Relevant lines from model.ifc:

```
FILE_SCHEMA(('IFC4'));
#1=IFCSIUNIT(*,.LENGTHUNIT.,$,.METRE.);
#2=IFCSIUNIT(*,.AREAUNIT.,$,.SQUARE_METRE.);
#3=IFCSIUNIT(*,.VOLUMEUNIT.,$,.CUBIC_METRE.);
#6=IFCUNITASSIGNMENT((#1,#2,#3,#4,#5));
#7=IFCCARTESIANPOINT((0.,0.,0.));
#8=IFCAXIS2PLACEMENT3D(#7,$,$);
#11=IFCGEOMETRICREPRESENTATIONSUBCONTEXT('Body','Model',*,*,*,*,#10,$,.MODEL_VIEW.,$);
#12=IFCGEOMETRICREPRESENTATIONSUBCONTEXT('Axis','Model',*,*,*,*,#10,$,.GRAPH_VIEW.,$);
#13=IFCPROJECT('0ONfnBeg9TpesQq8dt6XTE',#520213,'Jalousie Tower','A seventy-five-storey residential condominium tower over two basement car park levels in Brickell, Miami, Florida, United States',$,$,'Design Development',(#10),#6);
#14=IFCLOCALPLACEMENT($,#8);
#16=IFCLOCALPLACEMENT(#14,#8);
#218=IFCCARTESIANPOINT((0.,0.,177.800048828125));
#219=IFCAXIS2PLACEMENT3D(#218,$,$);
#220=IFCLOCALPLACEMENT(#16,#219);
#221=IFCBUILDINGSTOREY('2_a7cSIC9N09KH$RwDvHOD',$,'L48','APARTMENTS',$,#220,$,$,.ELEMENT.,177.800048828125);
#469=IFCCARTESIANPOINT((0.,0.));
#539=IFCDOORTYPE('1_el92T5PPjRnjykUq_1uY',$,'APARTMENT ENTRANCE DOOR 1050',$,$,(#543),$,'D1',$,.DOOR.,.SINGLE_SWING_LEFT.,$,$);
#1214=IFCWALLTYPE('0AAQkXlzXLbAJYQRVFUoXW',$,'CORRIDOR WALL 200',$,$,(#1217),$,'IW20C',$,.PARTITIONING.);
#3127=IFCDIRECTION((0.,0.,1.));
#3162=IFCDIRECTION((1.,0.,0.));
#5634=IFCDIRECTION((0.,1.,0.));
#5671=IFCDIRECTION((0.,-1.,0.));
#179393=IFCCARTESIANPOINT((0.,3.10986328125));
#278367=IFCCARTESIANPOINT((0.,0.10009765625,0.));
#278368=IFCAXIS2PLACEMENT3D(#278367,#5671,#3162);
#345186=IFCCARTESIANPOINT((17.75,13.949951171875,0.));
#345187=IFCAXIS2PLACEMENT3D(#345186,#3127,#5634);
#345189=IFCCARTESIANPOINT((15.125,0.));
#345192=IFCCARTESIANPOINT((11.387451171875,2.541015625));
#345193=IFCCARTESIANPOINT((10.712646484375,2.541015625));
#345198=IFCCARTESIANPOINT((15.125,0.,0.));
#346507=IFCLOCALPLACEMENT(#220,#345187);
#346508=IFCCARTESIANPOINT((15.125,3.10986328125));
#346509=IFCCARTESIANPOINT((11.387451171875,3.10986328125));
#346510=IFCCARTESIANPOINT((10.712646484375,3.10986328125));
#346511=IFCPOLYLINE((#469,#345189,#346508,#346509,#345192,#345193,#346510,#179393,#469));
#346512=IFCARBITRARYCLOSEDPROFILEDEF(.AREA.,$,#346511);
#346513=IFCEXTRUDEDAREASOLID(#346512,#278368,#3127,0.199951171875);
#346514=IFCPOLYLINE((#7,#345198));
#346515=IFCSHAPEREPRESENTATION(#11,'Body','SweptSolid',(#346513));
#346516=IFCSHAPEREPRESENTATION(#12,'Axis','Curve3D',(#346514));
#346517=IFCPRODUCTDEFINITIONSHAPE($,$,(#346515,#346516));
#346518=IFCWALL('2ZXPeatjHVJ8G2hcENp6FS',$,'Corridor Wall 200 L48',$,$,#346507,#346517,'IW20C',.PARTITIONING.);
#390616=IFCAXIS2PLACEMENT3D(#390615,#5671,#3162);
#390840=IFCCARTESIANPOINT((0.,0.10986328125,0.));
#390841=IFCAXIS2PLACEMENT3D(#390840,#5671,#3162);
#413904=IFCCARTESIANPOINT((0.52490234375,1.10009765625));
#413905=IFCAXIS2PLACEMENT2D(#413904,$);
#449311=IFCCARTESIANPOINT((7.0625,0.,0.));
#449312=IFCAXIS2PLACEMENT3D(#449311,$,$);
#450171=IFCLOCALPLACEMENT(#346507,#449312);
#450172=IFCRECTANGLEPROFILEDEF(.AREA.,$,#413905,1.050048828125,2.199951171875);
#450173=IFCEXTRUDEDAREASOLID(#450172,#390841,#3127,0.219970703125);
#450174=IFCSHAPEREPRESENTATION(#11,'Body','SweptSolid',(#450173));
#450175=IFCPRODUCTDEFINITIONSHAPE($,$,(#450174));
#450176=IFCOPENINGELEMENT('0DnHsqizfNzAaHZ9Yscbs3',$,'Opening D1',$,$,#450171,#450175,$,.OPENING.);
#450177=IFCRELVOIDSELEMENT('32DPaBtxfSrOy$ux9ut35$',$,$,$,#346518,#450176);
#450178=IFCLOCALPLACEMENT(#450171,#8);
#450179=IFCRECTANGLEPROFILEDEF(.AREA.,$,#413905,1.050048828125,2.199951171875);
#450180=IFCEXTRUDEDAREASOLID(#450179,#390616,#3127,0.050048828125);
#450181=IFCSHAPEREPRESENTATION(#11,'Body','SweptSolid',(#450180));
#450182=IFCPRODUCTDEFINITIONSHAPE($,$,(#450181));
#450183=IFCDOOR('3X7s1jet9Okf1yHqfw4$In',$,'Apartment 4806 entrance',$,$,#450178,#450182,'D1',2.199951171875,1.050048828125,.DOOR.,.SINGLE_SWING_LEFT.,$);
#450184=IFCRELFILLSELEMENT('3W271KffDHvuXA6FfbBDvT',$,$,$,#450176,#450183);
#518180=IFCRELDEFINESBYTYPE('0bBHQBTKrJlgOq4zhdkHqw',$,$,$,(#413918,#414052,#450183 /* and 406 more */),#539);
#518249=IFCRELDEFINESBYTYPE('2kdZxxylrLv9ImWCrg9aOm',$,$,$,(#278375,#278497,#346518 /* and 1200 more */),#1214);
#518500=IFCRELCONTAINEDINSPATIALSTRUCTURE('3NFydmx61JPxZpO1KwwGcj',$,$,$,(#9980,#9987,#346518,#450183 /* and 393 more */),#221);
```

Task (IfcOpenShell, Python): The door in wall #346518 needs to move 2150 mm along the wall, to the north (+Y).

```python
import ifcopenshell
import ifcopenshell.api.geometry
import ifcopenshell.util.placement

model = ifcopenshell.open("model.ifc")

door = model.by_id(450183)
opening = door.FillsVoids[0].RelatingOpeningElement
wall = opening.VoidsElements[0].RelatingBuildingElement

wall_matrix = ifcopenshell.util.placement.get_local_placement(wall.ObjectPlacement)
shift = wall_matrix[:3, 0] * 2.15
before = ifcopenshell.util.placement.get_local_placement(door.ObjectPlacement)[:3, 3].copy()

# The door is placed relative to its opening, so it follows when the opening moves.
matrix = ifcopenshell.util.placement.get_local_placement(opening.ObjectPlacement)
matrix[:3, 3] += shift
ifcopenshell.api.geometry.edit_object_placement(
    model, product=opening, matrix=matrix, is_si=False, should_transform_children=True
)

after = ifcopenshell.util.placement.get_local_placement(door.ObjectPlacement)[:3, 3]
print("door moved by", (after - before).round(3) + 0.0)

model.write("model_updated.ifc")
```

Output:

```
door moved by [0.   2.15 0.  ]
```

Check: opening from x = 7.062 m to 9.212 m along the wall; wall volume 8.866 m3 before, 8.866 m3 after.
